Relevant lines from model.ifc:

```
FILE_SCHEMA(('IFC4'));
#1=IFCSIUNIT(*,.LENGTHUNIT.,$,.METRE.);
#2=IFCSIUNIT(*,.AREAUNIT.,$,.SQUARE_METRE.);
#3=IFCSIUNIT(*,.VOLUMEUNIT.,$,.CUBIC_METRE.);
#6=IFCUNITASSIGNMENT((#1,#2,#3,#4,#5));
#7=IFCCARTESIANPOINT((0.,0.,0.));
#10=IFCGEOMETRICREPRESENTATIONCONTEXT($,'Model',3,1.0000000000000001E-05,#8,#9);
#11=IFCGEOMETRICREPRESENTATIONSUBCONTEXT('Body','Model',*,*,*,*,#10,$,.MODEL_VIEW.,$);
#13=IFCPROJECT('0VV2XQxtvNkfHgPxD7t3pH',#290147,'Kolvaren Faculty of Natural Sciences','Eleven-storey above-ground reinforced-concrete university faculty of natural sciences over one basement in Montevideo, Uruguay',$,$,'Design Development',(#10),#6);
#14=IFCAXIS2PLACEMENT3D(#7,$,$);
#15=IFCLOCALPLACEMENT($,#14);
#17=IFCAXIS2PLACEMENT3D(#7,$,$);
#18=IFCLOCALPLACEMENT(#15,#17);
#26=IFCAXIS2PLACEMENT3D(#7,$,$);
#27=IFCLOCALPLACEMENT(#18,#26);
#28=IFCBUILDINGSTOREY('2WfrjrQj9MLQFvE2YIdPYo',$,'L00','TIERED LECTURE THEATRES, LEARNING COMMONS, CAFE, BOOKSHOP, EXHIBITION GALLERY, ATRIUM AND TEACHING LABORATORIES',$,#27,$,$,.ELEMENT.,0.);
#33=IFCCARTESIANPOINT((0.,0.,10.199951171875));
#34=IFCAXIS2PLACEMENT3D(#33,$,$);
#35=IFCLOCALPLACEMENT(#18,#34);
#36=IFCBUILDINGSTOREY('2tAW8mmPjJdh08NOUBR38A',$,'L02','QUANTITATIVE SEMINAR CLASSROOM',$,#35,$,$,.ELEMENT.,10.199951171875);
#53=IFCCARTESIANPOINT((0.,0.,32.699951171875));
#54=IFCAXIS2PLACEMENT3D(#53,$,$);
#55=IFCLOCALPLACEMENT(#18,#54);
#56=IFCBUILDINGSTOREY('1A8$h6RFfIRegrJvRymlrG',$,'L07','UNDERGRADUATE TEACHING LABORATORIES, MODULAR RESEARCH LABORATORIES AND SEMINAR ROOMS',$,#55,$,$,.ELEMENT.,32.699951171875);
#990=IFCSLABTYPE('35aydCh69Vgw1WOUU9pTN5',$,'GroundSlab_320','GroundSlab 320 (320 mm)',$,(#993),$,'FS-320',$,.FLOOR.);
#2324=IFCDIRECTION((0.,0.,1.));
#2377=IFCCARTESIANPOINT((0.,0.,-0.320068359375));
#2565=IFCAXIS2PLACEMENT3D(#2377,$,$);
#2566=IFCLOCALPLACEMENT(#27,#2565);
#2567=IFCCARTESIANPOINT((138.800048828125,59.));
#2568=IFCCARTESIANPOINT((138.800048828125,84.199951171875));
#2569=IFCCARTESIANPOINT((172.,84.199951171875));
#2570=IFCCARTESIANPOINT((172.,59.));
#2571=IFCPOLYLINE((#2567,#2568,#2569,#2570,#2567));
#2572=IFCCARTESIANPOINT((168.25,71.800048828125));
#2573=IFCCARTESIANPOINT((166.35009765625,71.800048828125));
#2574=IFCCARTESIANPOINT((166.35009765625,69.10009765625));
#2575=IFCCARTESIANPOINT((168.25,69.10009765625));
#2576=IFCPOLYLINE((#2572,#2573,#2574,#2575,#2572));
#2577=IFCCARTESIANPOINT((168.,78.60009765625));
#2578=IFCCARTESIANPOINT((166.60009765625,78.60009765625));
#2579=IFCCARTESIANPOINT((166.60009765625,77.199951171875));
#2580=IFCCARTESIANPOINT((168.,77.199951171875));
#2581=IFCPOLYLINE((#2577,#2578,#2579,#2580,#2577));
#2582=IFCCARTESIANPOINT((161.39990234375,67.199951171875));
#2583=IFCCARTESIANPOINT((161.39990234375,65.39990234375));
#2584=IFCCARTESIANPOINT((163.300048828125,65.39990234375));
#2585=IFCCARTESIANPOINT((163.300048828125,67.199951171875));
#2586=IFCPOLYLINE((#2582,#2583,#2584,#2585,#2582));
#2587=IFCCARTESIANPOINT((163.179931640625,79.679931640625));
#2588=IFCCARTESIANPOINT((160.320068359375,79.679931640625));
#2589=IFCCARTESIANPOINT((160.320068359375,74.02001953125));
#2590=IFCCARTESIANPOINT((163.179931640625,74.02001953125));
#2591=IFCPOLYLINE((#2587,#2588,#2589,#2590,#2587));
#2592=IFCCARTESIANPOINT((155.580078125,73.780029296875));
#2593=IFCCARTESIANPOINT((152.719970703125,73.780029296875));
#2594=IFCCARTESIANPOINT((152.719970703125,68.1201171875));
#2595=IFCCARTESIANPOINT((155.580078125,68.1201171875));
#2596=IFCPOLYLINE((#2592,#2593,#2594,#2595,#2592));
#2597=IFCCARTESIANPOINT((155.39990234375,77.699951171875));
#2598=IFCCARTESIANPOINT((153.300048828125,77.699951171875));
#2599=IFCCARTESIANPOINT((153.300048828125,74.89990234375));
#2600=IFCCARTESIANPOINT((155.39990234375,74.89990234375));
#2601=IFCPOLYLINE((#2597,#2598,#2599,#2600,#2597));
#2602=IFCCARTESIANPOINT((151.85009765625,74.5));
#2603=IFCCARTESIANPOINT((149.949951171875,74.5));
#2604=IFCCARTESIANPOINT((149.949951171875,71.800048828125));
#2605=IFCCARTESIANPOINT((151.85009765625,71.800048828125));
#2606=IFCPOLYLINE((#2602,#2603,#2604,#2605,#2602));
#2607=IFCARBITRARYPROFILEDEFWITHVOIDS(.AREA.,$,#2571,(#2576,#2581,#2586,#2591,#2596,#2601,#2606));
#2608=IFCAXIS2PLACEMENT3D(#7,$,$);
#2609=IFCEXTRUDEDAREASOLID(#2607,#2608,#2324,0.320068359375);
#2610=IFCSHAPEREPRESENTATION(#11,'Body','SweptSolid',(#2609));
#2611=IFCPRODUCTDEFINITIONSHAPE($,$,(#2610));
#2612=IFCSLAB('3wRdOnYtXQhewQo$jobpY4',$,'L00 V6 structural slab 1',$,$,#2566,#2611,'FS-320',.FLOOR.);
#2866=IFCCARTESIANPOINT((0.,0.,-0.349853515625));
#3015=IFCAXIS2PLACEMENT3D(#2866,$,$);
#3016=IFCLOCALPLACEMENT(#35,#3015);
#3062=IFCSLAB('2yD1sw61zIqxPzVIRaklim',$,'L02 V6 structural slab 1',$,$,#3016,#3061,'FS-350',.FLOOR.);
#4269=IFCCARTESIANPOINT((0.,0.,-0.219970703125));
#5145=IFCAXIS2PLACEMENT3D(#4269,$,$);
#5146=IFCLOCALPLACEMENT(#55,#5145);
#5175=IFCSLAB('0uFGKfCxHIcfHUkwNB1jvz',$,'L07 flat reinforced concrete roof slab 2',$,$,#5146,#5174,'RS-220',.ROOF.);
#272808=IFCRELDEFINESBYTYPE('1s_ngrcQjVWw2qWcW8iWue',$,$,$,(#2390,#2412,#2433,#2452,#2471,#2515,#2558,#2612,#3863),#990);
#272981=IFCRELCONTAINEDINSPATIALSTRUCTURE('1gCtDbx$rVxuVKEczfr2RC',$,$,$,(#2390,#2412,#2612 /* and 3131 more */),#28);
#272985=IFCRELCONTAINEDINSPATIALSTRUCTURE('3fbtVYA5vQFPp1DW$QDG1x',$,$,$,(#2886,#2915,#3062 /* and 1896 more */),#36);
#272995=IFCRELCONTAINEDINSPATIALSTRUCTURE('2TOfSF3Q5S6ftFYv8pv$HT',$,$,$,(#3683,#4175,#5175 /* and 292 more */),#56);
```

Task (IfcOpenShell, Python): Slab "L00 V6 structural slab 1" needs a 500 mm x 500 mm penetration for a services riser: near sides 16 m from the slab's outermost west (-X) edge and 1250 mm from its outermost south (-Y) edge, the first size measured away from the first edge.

```python
import numpy as np
import ifcopenshell
import ifcopenshell.api.feature
import ifcopenshell.api.geometry
import ifcopenshell.api.root
import ifcopenshell.geom
import ifcopenshell.util.placement
import ifcopenshell.util.representation
import ifcopenshell.util.shape
import ifcopenshell.util.unit

model = ifcopenshell.open("model.ifc")
unit_scale = ifcopenshell.util.unit.calculate_unit_scale(model)
settings = ifcopenshell.geom.settings()


def volume(element):
    """Net volume in cubic metres, openings subtracted."""
    shape = ifcopenshell.geom.create_shape(settings, element)
    return ifcopenshell.util.shape.get_volume(shape.geometry)


slab = model.by_guid("3wRdOnYtXQhewQo$jobpY4")
before = volume(slab)

# Extent in the slab's own axes, in metres. The edges named are its -X and -Y sides.
slab_shape = ifcopenshell.geom.create_shape(settings, slab)
vertices = ifcopenshell.util.shape.get_vertices(slab_shape.geometry)
x_min, y_min, bottom = vertices.min(axis=0)
top = vertices[:, 2].max()

opening = ifcopenshell.api.root.create_entity(model, ifc_class="IfcOpeningElement", name="Services riser opening", predefined_type="OPENING")
context = ifcopenshell.util.representation.get_context(model, "Model", "Body", "MODEL_VIEW")
width, depth = 0.5, 0.5
outline = [(0.0, 0.0), (width, 0.0), (width, depth), (0.0, depth), (0.0, 0.0)]
# Overshoot both faces by 50 mm so the cut is clean.
shape = ifcopenshell.api.geometry.add_slab_representation(
    model, context=context, depth=top - bottom + 0.1, polyline=outline
)
ifcopenshell.api.geometry.assign_representation(model, product=opening, representation=shape)

matrix = ifcopenshell.util.placement.get_local_placement(slab.ObjectPlacement)
matrix[:, 3] = matrix @ np.append(np.array([x_min + 16, y_min + 1.25, bottom - 0.05]) / unit_scale, 1.0)
ifcopenshell.api.geometry.edit_object_placement(model, product=opening, matrix=matrix, is_si=False)
ifcopenshell.api.feature.add_feature(model, feature=opening, element=slab)

after = volume(slab)

print(f"slab volume {before:.3f} -> {after:.3f} m3")

model.write("model_edited.ifc")
```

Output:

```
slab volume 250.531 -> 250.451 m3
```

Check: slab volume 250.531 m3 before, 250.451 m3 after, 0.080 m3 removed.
